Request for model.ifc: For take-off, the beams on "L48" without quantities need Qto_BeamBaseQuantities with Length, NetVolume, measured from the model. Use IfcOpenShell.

First a look at what the model holds.

```python
import ifcopenshell
import ifcopenshell.util.element
import ifcopenshell.util.unit

model = ifcopenshell.open("model.ifc")
print(model.schema)
for unit_type in ("LENGTHUNIT", "AREAUNIT", "VOLUMEUNIT"):
    print(unit_type, ifcopenshell.util.unit.calculate_unit_scale(model, unit_type))
storey = next(s for s in model.by_type("IfcBuildingStorey") if s.Name == "L48")
beams = [e for e in ifcopenshell.util.element.get_decomposition(storey) if e.is_a("IfcBeam")]
for e in sorted(beams, key=lambda e: e.id()):
    print(e.id(), e.is_a(), e.Name, list(ifcopenshell.util.element.get_psets(e, qtos_only=True)), sep=" | ")
```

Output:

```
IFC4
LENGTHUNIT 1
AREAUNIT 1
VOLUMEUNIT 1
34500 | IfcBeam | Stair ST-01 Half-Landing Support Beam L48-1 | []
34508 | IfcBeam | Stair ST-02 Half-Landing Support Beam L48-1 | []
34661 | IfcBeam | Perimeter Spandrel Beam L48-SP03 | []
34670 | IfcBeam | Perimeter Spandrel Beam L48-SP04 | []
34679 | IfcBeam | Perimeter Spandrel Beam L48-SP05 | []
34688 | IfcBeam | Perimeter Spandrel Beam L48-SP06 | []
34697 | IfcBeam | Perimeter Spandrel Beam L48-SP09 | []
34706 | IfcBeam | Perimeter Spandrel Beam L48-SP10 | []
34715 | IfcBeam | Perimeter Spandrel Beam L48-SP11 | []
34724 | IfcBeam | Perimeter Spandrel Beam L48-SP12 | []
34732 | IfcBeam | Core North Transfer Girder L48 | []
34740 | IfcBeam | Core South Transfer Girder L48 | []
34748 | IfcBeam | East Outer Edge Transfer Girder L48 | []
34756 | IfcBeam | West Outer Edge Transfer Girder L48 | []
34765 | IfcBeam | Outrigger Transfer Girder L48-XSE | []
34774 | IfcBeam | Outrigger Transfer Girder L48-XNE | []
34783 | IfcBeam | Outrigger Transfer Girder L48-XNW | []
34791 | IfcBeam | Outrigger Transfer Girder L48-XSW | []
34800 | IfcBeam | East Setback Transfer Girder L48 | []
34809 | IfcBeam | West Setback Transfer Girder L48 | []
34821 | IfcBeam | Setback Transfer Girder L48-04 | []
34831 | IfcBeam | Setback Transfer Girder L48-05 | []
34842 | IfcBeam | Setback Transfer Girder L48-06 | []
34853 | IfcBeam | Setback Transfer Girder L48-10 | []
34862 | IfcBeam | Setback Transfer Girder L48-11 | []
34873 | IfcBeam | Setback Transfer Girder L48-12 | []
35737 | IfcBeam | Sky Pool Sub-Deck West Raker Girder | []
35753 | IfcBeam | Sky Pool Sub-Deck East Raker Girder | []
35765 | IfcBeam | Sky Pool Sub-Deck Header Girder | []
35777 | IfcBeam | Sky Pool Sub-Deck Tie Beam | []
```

```python
import ifcopenshell
import ifcopenshell.api.pset
import ifcopenshell.geom
import ifcopenshell.util.element
import ifcopenshell.util.shape
import ifcopenshell.util.unit

model = ifcopenshell.open("model.ifc")
unit_scale = ifcopenshell.util.unit.calculate_unit_scale(model)
volume_scale = ifcopenshell.util.unit.calculate_unit_scale(model, "VOLUMEUNIT")
settings = ifcopenshell.geom.settings()

storey = next(s for s in model.by_type("IfcBuildingStorey") if s.Name == "L48")
beams = [e for e in ifcopenshell.util.element.get_decomposition(storey) if e.is_a("IfcBeam")]

for e in sorted(beams, key=lambda e: e.id()):
    if ifcopenshell.util.element.get_psets(e, qtos_only=True, should_inherit=False):
        continue
    # Geometry comes back in metres, in the element's own axes.
    shape = ifcopenshell.geom.create_shape(settings, e)
    values = {
        "Length": ifcopenshell.util.shape.get_max_xyz(shape.geometry) / unit_scale,
        "NetVolume": ifcopenshell.util.shape.get_volume(shape.geometry) / volume_scale,
    }
    qto = ifcopenshell.api.pset.add_qto(model, product=e, name="Qto_BeamBaseQuantities")
    ifcopenshell.api.pset.edit_qto(model, qto=qto, properties=values)
    print(e.id(), {k: round(v, 3) for k, v in values.items()})

model.write("model_updated.ifc")
```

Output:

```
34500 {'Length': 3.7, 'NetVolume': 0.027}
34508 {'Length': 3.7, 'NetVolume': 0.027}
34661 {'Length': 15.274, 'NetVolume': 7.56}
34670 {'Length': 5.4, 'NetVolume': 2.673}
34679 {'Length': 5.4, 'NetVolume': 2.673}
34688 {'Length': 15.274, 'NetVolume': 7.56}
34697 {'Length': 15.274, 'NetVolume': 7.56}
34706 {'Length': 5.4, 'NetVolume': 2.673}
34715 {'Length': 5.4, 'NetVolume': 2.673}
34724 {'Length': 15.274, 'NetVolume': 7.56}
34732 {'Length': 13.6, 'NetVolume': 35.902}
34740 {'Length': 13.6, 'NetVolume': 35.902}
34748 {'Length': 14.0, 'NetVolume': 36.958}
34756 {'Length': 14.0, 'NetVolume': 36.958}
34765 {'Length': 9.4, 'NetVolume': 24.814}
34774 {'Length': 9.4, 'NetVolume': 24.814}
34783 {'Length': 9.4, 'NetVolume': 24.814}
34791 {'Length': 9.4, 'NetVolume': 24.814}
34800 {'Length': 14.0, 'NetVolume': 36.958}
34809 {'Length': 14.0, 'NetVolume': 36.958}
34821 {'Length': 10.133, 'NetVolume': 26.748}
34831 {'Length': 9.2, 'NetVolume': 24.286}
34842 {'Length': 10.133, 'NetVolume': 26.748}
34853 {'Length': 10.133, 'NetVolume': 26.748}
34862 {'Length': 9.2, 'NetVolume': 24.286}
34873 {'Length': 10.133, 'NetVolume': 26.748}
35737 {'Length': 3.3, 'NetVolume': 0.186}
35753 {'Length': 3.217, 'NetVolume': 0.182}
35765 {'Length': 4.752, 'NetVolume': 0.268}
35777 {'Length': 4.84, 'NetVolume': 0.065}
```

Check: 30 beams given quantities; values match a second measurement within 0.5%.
